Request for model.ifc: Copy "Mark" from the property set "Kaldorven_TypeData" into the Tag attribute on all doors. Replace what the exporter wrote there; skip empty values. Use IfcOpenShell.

First a look at what the model holds.

```python
import ifcopenshell
import ifcopenshell.util.element

model = ifcopenshell.open("model.ifc")
print(model.schema)
doors = model.by_type("IfcDoor")
print(len(doors), "doors")
for e in doors[:8]:
    source = ifcopenshell.util.element.get_pset(e, "Kaldorven_TypeData", "Mark")
    target = e.Tag
    print(e.id(), repr(source), repr(target), sep=" | ")
```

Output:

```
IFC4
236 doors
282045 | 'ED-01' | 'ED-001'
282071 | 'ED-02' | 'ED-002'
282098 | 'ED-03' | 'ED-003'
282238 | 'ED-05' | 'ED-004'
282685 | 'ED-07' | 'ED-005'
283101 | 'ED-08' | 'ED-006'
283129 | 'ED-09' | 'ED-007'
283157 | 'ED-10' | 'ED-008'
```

```python
import ifcopenshell
import ifcopenshell.util.element

model = ifcopenshell.open("model.ifc")

count = 0
for e in model.by_type("IfcDoor"):
    value = ifcopenshell.util.element.get_pset(e, "Kaldorven_TypeData", "Mark")
    current = e.Tag
    if not value or not value.strip() or current == value:
        continue
    e.Tag = value
    count += 1

print(count, "doors updated")

model.write("model_v2.ifc")
```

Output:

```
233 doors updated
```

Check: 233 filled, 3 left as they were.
